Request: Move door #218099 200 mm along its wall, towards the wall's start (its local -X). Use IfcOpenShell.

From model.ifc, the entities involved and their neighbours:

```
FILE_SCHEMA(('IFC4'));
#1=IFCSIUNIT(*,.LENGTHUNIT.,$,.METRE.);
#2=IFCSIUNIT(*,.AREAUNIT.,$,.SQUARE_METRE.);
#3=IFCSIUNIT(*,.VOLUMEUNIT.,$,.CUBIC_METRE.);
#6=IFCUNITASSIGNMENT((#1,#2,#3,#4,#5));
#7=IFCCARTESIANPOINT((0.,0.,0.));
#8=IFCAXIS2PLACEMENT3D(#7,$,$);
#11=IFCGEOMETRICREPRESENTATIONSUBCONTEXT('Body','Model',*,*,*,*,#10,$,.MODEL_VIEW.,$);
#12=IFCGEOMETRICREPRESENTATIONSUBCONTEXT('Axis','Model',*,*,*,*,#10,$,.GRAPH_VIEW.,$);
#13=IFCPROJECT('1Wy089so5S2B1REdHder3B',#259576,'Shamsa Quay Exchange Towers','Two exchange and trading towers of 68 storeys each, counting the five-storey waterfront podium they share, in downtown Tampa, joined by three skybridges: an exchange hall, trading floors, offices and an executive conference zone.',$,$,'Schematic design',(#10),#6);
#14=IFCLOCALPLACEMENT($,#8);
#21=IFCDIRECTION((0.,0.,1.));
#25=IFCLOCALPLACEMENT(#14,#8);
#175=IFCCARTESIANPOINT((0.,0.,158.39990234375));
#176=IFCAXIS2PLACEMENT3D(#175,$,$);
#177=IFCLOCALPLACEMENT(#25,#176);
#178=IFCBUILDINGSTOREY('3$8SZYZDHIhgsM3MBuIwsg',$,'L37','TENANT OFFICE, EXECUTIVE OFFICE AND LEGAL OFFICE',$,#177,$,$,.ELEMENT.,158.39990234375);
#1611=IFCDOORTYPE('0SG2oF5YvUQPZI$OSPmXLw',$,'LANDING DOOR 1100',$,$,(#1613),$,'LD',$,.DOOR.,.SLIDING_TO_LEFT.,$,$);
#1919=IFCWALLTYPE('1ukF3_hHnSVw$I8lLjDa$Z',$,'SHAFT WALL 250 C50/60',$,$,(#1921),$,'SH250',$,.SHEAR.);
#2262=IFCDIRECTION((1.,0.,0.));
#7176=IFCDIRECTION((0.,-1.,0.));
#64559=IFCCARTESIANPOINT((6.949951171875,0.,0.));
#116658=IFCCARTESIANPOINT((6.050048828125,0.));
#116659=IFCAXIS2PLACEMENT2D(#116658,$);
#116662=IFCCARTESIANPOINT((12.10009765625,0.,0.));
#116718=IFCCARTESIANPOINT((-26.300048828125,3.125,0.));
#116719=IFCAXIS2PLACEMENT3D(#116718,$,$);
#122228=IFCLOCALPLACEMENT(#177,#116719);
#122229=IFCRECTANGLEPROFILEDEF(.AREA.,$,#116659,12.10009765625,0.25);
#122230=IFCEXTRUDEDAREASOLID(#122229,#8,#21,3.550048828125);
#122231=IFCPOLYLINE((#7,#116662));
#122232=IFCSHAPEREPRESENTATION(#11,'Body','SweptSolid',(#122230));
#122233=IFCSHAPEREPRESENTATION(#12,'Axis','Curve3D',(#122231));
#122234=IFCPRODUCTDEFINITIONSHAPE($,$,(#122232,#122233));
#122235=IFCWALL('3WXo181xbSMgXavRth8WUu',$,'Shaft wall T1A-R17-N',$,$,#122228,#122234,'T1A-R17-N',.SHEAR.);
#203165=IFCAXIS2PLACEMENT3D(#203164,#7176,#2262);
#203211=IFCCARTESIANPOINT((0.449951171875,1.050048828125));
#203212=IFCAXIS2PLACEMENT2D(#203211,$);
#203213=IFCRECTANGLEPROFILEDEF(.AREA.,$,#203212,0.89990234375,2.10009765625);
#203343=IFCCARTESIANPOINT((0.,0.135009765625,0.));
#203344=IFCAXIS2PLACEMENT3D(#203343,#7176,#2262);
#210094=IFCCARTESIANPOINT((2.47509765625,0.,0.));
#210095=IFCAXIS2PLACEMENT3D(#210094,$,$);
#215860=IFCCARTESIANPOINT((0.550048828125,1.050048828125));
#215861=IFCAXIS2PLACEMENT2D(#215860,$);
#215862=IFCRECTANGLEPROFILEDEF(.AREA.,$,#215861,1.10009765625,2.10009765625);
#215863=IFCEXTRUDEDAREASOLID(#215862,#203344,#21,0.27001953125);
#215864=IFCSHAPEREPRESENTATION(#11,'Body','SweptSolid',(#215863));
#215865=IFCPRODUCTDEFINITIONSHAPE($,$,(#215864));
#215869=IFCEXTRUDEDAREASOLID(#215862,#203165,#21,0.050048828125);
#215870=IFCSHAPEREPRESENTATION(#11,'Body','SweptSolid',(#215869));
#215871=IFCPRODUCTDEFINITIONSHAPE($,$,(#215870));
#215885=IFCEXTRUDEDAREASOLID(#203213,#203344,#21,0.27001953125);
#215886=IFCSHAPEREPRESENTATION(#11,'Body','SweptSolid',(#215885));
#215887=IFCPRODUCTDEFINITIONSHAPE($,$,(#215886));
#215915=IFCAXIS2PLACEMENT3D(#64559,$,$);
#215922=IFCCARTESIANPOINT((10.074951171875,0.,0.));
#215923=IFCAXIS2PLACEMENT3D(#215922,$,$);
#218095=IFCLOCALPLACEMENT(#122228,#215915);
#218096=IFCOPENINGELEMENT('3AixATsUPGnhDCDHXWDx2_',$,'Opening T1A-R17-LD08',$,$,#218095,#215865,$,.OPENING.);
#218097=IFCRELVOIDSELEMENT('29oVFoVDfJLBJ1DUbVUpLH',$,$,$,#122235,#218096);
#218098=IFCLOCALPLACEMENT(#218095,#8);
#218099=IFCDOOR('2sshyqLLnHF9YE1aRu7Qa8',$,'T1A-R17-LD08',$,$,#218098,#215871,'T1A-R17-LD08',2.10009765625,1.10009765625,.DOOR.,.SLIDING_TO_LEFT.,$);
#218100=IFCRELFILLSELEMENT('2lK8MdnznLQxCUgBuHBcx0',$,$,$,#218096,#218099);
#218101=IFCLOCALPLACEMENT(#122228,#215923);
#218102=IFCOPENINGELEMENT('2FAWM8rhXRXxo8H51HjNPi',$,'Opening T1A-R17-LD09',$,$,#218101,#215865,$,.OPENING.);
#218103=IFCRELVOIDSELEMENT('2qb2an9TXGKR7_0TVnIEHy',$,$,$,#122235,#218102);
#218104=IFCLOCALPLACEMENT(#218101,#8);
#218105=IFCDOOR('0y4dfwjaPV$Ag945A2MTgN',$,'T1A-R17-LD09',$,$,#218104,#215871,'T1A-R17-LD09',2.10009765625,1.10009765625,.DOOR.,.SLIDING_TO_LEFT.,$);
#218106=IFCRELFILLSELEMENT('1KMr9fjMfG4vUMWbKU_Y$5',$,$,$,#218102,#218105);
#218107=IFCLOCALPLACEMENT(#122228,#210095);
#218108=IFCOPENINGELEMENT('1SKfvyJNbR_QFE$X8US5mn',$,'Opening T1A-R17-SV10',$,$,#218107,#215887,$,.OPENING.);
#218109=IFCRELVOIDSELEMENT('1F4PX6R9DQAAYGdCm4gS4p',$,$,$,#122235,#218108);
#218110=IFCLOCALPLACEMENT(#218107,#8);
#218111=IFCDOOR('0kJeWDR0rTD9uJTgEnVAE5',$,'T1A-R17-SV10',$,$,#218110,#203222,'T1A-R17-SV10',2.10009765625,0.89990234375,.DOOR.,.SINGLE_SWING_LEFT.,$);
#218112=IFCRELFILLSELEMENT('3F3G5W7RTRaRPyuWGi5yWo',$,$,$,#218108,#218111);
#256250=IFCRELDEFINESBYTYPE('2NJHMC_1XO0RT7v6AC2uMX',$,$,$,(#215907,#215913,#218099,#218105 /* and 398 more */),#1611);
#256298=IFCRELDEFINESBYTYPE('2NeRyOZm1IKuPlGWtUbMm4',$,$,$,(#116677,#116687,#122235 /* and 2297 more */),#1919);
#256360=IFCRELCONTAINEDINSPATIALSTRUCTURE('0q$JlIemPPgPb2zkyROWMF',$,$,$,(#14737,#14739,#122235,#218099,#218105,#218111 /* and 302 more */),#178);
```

```python
import ifcopenshell
import ifcopenshell.api.geometry
import ifcopenshell.util.placement
import ifcopenshell.util.unit

model = ifcopenshell.open("model.ifc")
unit_scale = ifcopenshell.util.unit.calculate_unit_scale(model)

door = model.by_guid("2sshyqLLnHF9YE1aRu7Qa8")
opening = door.FillsVoids[0].RelatingOpeningElement
wall = opening.VoidsElements[0].RelatingBuildingElement

wall_matrix = ifcopenshell.util.placement.get_local_placement(wall.ObjectPlacement)
shift = wall_matrix[:3, 0] * -0.2 / unit_scale
before = ifcopenshell.util.placement.get_local_placement(door.ObjectPlacement)[:3, 3].copy()

# The door is placed relative to its opening, so it follows when the opening moves.
matrix = ifcopenshell.util.placement.get_local_placement(opening.ObjectPlacement)
matrix[:3, 3] += shift
ifcopenshell.api.geometry.edit_object_placement(
    model, product=opening, matrix=matrix, is_si=False, should_transform_children=True
)

after = ifcopenshell.util.placement.get_local_placement(door.ObjectPlacement)[:3, 3]
print("door moved by", (after - before).round(3) + 0.0)

model.write("model_v2.ifc")
```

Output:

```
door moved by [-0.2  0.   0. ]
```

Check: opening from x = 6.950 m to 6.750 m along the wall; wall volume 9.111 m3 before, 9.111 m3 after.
